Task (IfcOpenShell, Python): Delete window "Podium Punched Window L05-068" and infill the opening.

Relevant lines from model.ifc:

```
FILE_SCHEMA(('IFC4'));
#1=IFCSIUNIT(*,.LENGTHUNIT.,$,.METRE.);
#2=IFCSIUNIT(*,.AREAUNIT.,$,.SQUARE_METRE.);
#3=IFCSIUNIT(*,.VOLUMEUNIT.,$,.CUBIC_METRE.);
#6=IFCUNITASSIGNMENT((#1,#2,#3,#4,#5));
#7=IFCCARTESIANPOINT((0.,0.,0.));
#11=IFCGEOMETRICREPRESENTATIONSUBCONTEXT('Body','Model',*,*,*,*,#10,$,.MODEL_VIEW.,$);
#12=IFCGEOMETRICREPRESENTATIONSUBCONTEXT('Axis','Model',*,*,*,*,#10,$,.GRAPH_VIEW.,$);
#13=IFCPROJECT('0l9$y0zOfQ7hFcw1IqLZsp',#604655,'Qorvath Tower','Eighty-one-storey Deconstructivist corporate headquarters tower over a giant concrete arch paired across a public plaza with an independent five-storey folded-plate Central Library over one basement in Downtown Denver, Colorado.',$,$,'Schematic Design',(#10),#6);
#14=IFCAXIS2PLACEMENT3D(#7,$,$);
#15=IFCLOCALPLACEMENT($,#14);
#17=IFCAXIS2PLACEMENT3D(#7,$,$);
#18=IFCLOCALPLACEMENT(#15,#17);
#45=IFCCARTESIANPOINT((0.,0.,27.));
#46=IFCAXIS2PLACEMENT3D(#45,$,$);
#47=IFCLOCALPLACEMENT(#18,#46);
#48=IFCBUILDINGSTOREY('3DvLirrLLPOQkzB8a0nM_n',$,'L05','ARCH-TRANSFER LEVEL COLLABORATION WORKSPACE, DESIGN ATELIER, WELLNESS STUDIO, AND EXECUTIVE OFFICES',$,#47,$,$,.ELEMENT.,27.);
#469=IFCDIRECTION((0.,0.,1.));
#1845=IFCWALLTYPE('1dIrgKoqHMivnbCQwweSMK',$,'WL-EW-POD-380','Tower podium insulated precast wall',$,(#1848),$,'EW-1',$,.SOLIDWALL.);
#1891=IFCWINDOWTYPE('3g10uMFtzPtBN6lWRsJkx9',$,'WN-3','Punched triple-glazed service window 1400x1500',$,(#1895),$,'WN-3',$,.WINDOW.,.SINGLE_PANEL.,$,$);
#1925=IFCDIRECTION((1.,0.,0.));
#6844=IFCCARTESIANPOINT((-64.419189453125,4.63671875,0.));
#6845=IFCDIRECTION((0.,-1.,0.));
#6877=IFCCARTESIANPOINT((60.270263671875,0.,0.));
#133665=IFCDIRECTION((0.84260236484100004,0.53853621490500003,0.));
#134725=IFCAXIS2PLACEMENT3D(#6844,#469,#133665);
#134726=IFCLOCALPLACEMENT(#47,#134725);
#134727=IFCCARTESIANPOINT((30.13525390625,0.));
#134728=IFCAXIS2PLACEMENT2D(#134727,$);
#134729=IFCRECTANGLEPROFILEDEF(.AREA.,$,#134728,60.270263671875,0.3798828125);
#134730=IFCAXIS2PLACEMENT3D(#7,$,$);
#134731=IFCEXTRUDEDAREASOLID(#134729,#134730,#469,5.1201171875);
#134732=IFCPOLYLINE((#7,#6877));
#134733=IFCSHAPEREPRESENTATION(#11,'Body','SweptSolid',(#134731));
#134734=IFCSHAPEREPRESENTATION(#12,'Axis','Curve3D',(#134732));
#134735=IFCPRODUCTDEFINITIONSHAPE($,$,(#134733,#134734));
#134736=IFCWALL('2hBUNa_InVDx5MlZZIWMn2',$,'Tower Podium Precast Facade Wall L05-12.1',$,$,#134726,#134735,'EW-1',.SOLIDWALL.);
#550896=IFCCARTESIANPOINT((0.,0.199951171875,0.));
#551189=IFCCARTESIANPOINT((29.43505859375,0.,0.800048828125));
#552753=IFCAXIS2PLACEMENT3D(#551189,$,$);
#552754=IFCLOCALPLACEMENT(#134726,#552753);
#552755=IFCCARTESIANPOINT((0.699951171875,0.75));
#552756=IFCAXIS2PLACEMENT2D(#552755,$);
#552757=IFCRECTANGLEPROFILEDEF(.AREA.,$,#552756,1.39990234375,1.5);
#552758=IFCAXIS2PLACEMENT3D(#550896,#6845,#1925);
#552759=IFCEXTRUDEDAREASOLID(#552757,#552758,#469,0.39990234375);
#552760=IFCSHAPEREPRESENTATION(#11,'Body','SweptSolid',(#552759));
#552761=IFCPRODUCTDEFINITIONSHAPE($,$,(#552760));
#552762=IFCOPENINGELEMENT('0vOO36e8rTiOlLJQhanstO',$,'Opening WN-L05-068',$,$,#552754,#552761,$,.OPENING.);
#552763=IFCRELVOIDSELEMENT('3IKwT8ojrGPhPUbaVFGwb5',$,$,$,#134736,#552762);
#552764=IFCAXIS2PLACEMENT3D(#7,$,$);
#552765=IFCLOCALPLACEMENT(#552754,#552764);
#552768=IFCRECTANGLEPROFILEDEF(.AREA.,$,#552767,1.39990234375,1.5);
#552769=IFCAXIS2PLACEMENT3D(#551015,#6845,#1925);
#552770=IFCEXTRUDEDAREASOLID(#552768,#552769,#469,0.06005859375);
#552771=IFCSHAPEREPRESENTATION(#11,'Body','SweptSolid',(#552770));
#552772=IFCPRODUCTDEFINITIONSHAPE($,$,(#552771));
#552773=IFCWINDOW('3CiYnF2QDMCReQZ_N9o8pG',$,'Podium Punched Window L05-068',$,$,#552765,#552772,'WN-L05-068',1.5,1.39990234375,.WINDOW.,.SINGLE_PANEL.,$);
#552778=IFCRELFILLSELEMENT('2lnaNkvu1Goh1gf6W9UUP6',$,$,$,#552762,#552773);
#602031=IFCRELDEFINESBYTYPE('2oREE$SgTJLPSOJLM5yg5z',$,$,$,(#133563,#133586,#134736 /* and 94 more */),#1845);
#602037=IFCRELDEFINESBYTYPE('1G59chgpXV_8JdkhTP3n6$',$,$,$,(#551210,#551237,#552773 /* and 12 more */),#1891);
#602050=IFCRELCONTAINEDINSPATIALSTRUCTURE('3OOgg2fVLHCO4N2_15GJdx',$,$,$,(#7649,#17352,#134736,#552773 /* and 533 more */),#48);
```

```python
import ifcopenshell
import ifcopenshell.api.feature
import ifcopenshell.api.root
import ifcopenshell.geom
import ifcopenshell.util.shape

model = ifcopenshell.open("model.ifc")
settings = ifcopenshell.geom.settings()


def volume(element):
    """Net volume in cubic metres, openings subtracted."""
    shape = ifcopenshell.geom.create_shape(settings, element)
    return ifcopenshell.util.shape.get_volume(shape.geometry)


window = model.by_guid("3CiYnF2QDMCReQZ_N9o8pG")
opening = window.FillsVoids[0].RelatingOpeningElement
wall = opening.VoidsElements[0].RelatingBuildingElement
before = volume(wall)

ifcopenshell.api.root.remove_product(model, product=window)
ifcopenshell.api.feature.remove_feature(model, feature=opening)

after = volume(wall)

print(f"wall volume {before:.3f} -> {after:.3f} m3")

model.write("model_updated.ifc")
```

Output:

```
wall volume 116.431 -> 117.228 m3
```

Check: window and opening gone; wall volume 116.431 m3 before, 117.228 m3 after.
